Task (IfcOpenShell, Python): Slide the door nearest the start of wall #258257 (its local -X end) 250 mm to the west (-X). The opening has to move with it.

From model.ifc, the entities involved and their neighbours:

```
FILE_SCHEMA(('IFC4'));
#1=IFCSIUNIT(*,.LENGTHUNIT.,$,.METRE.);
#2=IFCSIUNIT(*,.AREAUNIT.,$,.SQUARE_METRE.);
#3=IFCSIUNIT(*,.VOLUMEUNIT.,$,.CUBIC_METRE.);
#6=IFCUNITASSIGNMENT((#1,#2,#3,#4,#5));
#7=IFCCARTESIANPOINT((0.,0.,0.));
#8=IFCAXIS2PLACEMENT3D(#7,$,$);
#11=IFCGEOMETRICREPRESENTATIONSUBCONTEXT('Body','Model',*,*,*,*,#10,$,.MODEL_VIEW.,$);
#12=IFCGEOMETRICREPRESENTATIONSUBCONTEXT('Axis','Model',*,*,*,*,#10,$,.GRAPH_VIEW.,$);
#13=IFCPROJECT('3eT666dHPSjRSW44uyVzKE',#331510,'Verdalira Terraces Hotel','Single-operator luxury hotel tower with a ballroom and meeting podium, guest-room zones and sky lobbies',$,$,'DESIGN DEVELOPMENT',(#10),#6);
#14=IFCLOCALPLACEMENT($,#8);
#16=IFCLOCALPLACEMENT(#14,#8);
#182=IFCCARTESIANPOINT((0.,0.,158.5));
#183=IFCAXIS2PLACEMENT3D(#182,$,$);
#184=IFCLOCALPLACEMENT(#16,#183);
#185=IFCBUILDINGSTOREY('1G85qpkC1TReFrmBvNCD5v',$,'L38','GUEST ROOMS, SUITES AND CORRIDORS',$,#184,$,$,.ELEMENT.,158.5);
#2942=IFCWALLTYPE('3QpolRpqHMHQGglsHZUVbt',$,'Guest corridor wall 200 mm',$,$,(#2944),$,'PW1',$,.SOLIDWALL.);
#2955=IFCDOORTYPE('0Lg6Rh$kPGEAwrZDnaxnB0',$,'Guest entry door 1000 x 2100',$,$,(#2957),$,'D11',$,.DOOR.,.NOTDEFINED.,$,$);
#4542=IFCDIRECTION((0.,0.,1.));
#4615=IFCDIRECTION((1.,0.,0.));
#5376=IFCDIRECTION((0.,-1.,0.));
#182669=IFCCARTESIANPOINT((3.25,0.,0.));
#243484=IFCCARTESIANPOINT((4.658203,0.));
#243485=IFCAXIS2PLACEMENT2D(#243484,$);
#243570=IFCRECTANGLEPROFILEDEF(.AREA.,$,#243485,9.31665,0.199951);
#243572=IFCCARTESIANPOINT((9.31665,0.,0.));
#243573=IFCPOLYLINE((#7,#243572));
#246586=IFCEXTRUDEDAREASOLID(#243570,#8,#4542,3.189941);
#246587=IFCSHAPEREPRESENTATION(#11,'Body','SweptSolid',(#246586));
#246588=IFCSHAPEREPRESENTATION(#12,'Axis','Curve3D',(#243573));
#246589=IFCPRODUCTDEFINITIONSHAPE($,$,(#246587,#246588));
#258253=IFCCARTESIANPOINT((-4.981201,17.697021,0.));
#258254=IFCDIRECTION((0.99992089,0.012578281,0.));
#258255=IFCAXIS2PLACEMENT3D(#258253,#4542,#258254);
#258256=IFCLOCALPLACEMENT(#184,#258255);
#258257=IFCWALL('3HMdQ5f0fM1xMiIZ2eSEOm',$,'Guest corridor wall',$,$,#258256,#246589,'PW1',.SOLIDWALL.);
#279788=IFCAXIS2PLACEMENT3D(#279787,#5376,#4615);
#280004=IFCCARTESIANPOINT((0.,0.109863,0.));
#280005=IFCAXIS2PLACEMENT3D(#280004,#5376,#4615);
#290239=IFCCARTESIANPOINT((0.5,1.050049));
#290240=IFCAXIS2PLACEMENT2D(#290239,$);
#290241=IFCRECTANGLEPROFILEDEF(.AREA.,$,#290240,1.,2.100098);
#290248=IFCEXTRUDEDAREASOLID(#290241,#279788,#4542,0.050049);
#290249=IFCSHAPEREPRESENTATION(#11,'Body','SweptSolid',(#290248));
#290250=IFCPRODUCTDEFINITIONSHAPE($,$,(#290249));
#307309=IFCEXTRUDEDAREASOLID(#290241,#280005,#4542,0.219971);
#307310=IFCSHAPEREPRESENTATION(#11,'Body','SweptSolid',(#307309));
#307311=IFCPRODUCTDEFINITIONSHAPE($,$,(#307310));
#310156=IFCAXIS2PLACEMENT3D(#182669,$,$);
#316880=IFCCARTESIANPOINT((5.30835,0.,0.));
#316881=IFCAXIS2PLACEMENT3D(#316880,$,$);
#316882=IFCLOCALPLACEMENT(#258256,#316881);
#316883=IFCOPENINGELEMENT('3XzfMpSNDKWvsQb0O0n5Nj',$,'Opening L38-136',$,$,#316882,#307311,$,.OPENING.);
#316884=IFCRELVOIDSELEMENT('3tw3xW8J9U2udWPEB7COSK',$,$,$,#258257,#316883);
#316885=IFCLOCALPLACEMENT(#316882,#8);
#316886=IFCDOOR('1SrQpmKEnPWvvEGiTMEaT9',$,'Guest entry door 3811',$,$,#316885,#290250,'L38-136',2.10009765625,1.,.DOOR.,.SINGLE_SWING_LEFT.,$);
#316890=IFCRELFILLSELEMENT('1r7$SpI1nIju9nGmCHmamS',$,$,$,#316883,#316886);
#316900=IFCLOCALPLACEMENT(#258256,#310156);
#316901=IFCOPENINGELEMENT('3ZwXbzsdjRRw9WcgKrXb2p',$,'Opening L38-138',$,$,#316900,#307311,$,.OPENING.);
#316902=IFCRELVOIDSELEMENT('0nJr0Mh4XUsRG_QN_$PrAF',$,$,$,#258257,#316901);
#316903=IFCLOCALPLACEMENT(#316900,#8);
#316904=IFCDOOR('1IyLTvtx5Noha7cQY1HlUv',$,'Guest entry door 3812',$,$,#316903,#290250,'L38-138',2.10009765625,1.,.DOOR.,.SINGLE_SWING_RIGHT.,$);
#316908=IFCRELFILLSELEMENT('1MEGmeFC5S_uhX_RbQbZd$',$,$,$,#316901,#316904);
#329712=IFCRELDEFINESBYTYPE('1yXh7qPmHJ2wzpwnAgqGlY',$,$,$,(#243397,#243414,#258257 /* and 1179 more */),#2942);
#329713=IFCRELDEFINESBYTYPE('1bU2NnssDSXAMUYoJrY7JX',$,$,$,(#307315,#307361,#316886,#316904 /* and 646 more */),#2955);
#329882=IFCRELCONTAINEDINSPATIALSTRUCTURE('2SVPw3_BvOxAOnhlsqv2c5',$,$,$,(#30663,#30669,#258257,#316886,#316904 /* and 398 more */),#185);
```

```python
import ifcopenshell
import ifcopenshell.api.geometry
import ifcopenshell.util.placement
import ifcopenshell.util.unit

model = ifcopenshell.open("model.ifc")
unit_scale = ifcopenshell.util.unit.calculate_unit_scale(model)

door = model.by_guid("1IyLTvtx5Noha7cQY1HlUv")
opening = door.FillsVoids[0].RelatingOpeningElement
wall = opening.VoidsElements[0].RelatingBuildingElement

wall_matrix = ifcopenshell.util.placement.get_local_placement(wall.ObjectPlacement)
shift = wall_matrix[:3, 0] * -0.25 / unit_scale
before = ifcopenshell.util.placement.get_local_placement(door.ObjectPlacement)[:3, 3].copy()

# The door is placed relative to its opening, so it follows when the opening moves.
matrix = ifcopenshell.util.placement.get_local_placement(opening.ObjectPlacement)
matrix[:3, 3] += shift
ifcopenshell.api.geometry.edit_object_placement(
    model, product=opening, matrix=matrix, is_si=False, should_transform_children=True
)

after = ifcopenshell.util.placement.get_local_placement(door.ObjectPlacement)[:3, 3]
print("door moved by", (after - before).round(3) + 0.0)

model.write("model_edited.ifc")
```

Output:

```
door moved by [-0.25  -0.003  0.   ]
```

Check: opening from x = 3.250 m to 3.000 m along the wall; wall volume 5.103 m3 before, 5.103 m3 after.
